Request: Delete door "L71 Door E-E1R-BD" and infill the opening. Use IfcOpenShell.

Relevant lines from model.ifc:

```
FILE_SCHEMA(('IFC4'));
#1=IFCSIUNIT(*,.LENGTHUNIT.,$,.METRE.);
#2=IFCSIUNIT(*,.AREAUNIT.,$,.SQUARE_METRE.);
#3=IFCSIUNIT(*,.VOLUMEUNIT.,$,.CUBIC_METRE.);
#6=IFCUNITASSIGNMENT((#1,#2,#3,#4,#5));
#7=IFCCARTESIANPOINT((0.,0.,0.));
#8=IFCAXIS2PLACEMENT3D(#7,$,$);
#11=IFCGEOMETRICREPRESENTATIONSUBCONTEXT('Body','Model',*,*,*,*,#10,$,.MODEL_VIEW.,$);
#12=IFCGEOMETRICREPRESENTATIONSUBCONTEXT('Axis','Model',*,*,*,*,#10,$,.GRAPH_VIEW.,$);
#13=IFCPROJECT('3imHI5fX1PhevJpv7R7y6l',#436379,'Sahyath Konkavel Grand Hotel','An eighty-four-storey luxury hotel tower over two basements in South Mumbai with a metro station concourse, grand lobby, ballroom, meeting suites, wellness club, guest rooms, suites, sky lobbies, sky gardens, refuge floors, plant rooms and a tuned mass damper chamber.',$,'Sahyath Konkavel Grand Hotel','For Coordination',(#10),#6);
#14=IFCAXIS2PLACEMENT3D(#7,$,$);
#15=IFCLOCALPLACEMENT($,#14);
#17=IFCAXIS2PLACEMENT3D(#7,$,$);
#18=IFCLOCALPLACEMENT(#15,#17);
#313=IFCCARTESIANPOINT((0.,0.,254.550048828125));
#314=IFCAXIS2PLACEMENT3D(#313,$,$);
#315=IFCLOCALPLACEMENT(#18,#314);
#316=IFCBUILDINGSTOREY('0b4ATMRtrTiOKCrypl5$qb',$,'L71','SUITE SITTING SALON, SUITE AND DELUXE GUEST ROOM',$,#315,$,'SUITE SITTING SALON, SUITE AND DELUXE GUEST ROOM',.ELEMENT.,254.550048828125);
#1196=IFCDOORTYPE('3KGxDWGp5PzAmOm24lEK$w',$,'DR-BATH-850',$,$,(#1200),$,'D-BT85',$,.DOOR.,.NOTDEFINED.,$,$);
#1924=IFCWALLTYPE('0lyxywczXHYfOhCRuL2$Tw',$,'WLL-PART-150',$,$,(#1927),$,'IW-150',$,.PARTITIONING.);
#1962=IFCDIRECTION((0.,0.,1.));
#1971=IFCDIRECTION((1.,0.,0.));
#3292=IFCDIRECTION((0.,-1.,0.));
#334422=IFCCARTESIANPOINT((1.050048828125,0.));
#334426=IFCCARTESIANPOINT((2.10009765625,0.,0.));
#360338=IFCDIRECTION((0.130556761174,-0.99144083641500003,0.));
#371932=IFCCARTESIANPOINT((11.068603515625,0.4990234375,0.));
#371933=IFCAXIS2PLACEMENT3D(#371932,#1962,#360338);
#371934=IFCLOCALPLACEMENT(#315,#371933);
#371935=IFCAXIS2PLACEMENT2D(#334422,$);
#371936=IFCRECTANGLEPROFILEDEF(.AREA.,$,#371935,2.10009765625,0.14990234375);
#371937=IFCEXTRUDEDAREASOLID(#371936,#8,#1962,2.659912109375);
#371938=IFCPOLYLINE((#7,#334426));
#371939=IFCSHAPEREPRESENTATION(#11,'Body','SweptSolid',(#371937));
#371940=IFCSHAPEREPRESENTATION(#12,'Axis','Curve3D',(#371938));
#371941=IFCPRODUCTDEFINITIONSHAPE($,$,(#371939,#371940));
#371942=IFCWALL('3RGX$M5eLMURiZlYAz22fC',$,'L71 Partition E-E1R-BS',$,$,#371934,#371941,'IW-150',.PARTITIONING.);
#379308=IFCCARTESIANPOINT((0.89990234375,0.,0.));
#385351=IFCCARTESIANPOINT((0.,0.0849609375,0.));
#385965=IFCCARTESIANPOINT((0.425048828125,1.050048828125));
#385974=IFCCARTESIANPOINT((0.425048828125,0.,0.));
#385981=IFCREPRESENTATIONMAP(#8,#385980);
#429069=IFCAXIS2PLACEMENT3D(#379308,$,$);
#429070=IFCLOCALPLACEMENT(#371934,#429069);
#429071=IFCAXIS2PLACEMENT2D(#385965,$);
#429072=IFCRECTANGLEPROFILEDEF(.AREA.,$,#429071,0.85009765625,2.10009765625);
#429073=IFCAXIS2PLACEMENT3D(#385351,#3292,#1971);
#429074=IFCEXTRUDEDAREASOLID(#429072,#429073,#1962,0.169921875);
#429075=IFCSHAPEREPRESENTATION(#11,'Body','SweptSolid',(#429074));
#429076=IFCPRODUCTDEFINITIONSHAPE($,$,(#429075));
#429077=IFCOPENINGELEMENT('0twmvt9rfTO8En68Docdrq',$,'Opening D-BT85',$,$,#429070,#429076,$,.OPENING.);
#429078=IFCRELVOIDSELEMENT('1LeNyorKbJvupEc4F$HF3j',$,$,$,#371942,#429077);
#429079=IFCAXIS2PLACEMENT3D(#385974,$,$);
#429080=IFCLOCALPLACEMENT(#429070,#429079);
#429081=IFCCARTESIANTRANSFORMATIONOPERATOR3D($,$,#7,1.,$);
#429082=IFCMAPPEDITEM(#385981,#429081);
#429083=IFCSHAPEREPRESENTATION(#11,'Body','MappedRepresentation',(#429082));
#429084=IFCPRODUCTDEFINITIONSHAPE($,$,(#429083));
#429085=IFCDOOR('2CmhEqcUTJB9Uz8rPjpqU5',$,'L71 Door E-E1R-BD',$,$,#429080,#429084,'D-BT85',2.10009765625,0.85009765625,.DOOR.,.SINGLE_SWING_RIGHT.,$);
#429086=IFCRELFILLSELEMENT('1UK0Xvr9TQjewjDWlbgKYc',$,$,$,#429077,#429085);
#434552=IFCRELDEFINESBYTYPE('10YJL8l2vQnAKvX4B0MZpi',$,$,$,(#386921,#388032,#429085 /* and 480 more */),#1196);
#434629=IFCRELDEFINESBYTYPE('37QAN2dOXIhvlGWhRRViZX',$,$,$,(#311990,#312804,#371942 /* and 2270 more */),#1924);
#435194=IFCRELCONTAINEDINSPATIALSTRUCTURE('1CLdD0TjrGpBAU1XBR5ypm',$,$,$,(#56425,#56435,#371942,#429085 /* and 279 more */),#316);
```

```python
import ifcopenshell
import ifcopenshell.api.feature
import ifcopenshell.api.root
import ifcopenshell.geom
import ifcopenshell.util.shape

model = ifcopenshell.open("model.ifc")
settings = ifcopenshell.geom.settings()


def volume(element):
    """Net volume in cubic metres, openings subtracted."""
    shape = ifcopenshell.geom.create_shape(settings, element)
    return ifcopenshell.util.shape.get_volume(shape.geometry)


door = model.by_guid("2CmhEqcUTJB9Uz8rPjpqU5")
opening = door.FillsVoids[0].RelatingOpeningElement
wall = opening.VoidsElements[0].RelatingBuildingElement
before = volume(wall)

ifcopenshell.api.root.remove_product(model, product=door)
ifcopenshell.api.feature.remove_feature(model, feature=opening)

after = volume(wall)

print(f"wall volume {before:.3f} -> {after:.3f} m3")

model.write("model_edited.ifc")
```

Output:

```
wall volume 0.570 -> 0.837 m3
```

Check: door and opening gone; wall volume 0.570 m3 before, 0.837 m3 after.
